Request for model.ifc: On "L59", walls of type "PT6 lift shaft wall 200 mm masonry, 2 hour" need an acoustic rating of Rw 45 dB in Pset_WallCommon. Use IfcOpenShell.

First a look at what the model holds.

```python
import ifcopenshell
import ifcopenshell.util.element

model = ifcopenshell.open("model.ifc")
print(model.schema)
storey = next(s for s in model.by_type("IfcBuildingStorey") if s.Name == "L59")
walls = [e for e in ifcopenshell.util.element.get_decomposition(storey) if e.is_a("IfcWall")]
seen = {}
for e in walls:
    element_type = ifcopenshell.util.element.get_type(e)
    key = (element_type.Name if element_type != e and element_type else None, ifcopenshell.util.element.get_pset(e, "Pset_WallCommon", "AcousticRating"))
    seen[key] = seen.get(key, 0) + 1
for (name, value), count in sorted(seen.items(), key=str):
    print(count, "x", name, "|", value)
```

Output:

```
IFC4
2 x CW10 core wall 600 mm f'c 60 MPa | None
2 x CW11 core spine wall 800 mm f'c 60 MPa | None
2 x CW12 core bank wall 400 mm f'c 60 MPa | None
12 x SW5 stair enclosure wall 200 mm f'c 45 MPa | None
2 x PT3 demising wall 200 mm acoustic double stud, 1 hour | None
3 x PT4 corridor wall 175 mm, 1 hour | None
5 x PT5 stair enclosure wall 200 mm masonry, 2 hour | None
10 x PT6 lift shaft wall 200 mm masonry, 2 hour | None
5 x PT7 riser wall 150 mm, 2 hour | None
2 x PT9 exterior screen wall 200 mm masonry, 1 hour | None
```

```python
import ifcopenshell
import ifcopenshell.api.pset
import ifcopenshell.util.element

model = ifcopenshell.open("model.ifc")

storey = next(s for s in model.by_type("IfcBuildingStorey") if s.Name == "L59")
walls = [e for e in ifcopenshell.util.element.get_decomposition(storey) if e.is_a("IfcWall")]

count = 0
for e in walls:
    element_type = ifcopenshell.util.element.get_type(e)
    if element_type in (None, e) or element_type.Name != "PT6 lift shaft wall 200 mm masonry, 2 hour":
        continue
    found = ifcopenshell.util.element.get_pset(e, "Pset_WallCommon", should_inherit=False)
    if found:
        pset = model.by_id(found["id"])
        if len(ifcopenshell.util.element.get_elements_by_pset(pset)) > 1:
            pset = ifcopenshell.api.pset.unshare_pset(model, products=[e], pset=pset)[0]
    else:
        pset = ifcopenshell.api.pset.add_pset(model, product=e, name="Pset_WallCommon")
    ifcopenshell.api.pset.edit_pset(model, pset=pset, properties={"AcousticRating": "Rw 45 dB"})
    count += 1

print(count, "walls updated")

model.write("model_updated.ifc")
```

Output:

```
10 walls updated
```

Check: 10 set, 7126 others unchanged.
